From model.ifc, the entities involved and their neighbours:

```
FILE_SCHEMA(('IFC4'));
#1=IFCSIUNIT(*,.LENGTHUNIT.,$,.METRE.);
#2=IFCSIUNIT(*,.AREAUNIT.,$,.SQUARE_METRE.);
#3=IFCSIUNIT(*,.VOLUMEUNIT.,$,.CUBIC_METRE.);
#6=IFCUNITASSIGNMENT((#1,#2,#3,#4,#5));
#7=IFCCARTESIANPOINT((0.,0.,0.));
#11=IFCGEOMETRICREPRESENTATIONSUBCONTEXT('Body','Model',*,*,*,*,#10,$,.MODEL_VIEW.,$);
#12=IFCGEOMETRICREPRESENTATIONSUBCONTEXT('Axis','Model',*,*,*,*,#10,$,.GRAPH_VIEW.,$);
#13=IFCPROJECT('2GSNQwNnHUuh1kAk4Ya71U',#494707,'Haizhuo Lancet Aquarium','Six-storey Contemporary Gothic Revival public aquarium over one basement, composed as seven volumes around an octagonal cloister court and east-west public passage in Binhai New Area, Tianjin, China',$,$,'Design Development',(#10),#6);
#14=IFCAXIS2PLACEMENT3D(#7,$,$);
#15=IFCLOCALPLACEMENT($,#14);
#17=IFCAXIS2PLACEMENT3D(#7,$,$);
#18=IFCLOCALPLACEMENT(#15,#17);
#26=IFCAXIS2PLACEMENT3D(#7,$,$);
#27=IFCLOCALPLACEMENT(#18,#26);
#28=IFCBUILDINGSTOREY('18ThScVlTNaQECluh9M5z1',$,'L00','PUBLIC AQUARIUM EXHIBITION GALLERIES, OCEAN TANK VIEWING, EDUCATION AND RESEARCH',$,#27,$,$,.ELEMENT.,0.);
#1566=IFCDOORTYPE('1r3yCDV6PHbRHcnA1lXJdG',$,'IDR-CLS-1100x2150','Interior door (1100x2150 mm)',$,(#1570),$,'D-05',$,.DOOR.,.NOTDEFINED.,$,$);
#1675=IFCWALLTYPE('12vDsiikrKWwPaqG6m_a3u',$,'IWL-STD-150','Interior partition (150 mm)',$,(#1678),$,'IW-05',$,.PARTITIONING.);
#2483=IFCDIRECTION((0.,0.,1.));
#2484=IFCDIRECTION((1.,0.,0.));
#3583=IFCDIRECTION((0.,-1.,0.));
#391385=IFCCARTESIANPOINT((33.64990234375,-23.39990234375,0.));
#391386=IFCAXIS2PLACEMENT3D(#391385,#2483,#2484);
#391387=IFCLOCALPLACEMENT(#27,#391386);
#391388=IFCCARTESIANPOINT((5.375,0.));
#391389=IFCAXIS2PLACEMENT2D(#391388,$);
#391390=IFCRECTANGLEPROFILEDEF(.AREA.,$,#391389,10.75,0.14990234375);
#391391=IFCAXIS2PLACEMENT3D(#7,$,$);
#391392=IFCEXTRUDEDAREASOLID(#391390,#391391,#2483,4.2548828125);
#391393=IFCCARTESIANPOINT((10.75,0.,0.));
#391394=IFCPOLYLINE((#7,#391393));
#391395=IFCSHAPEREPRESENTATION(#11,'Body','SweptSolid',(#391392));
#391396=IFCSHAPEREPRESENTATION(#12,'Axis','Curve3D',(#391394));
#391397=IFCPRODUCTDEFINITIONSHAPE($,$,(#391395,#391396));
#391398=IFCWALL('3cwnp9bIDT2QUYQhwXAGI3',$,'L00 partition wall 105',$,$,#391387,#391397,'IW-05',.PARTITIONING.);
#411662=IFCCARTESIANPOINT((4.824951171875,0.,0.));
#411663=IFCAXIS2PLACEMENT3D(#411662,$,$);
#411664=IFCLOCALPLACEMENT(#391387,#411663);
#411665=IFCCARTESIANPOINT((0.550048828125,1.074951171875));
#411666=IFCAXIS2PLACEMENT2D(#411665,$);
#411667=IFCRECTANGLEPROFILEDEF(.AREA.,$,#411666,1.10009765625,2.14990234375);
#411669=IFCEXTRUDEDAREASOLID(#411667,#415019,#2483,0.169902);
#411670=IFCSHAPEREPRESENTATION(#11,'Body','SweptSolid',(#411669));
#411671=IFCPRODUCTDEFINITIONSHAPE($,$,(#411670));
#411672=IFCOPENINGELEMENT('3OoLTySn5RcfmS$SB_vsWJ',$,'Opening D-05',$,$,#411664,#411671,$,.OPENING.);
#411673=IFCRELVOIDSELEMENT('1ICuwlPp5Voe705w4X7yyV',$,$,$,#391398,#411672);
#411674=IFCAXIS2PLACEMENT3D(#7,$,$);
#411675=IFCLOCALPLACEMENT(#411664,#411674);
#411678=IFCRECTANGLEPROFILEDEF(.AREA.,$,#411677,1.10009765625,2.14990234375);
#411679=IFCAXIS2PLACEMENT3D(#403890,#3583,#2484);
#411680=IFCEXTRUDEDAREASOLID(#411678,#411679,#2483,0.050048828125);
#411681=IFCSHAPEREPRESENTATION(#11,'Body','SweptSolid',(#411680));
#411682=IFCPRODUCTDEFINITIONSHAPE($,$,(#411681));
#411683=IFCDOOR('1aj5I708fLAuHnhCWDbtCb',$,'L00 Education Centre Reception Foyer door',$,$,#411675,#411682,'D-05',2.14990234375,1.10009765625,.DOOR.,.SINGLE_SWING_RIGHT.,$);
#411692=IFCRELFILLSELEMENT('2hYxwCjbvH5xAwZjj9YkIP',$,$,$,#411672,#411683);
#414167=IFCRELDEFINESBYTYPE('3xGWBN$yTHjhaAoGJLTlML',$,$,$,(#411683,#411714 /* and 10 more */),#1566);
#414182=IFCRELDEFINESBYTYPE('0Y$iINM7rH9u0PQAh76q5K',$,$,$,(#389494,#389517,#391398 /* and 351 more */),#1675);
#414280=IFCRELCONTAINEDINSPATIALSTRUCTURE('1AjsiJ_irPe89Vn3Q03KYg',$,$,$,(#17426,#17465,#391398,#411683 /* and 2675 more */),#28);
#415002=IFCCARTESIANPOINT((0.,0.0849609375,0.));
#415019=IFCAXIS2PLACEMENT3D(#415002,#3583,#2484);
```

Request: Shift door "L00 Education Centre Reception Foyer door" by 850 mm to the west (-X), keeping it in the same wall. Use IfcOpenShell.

```python
import ifcopenshell
import ifcopenshell.api.geometry
import ifcopenshell.util.placement
import ifcopenshell.util.unit

model = ifcopenshell.open("model.ifc")
unit_scale = ifcopenshell.util.unit.calculate_unit_scale(model)

door = model.by_id(411683)
opening = door.FillsVoids[0].RelatingOpeningElement
wall = opening.VoidsElements[0].RelatingBuildingElement

wall_matrix = ifcopenshell.util.placement.get_local_placement(wall.ObjectPlacement)
shift = wall_matrix[:3, 0] * -0.85 / unit_scale
before = ifcopenshell.util.placement.get_local_placement(door.ObjectPlacement)[:3, 3].copy()

# The door is placed relative to its opening, so it follows when the opening moves.
matrix = ifcopenshell.util.placement.get_local_placement(opening.ObjectPlacement)
matrix[:3, 3] += shift
ifcopenshell.api.geometry.edit_object_placement(
    model, product=opening, matrix=matrix, is_si=False, should_transform_children=True
)

after = ifcopenshell.util.placement.get_local_placement(door.ObjectPlacement)[:3, 3]
print("door moved by", (after - before).round(3) + 0.0)

model.write("model_edited.ifc")
```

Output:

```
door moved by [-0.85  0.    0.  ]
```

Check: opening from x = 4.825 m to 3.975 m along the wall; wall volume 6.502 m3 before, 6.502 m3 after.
